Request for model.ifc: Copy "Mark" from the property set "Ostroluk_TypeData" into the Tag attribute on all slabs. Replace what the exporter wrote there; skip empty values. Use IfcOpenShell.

First a look at what the model holds.

```python
import ifcopenshell
import ifcopenshell.util.element

model = ifcopenshell.open("model.ifc")
print(model.schema)
slabs = model.by_type("IfcSlab")
print(len(slabs), "slabs")
for e in slabs[:8]:
    source = ifcopenshell.util.element.get_pset(e, "Ostroluk_TypeData", "Mark")
    target = e.Tag
    print(e.id(), repr(source), repr(target), sep=" | ")
```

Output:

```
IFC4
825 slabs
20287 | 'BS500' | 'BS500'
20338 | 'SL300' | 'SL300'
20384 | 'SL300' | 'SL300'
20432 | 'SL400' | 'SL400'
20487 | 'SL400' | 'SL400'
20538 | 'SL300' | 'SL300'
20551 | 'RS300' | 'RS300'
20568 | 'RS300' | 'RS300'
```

```python
import ifcopenshell
import ifcopenshell.util.element

model = ifcopenshell.open("model.ifc")

count = 0
for e in model.by_type("IfcSlab"):
    value = ifcopenshell.util.element.get_pset(e, "Ostroluk_TypeData", "Mark")
    current = e.Tag
    if not value or not value.strip() or current == value:
        continue
    e.Tag = value
    count += 1

print(count, "slabs updated")

model.write("model_edited.ifc")
```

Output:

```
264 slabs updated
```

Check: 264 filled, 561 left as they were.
